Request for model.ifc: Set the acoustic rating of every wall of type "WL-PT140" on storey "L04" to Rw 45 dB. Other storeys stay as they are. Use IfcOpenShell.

First a look at what the model holds.

```python
import ifcopenshell
import ifcopenshell.util.element

model = ifcopenshell.open("model.ifc")
print(model.schema)
storey = next(s for s in model.by_type("IfcBuildingStorey") if s.Name == "L04")
walls = [e for e in ifcopenshell.util.element.get_decomposition(storey) if e.is_a("IfcWall")]
seen = {}
for e in walls:
    element_type = ifcopenshell.util.element.get_type(e)
    key = (element_type.Name if element_type != e and element_type else None, ifcopenshell.util.element.get_pset(e, "Pset_WallCommon", "AcousticRating"))
    seen[key] = seen.get(key, 0) + 1
for (name, value), count in sorted(seen.items(), key=str):
    print(count, "x", name, "|", value)
```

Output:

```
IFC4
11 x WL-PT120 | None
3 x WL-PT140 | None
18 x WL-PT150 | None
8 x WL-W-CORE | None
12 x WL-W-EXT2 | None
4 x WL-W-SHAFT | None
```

```python
import ifcopenshell
import ifcopenshell.api.pset
import ifcopenshell.util.element

model = ifcopenshell.open("model.ifc")

storey = next(s for s in model.by_type("IfcBuildingStorey") if s.Name == "L04")
walls = [e for e in ifcopenshell.util.element.get_decomposition(storey) if e.is_a("IfcWall")]

count = 0
for e in walls:
    element_type = ifcopenshell.util.element.get_type(e)
    if element_type in (None, e) or element_type.Name != "WL-PT140":
        continue
    # add_pset returns the element's existing set when there is one.
    pset = ifcopenshell.api.pset.add_pset(model, product=e, name="Pset_WallCommon")
    ifcopenshell.api.pset.edit_pset(model, pset=pset, properties={"AcousticRating": "Rw 45 dB"})
    count += 1

print(count, "walls updated")

model.write("model_edited.ifc")
```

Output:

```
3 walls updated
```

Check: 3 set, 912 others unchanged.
